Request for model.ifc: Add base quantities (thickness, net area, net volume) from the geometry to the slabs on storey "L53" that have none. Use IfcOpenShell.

First a look at what the model holds.

```python
import ifcopenshell
import ifcopenshell.util.element
import ifcopenshell.util.unit

model = ifcopenshell.open("model.ifc")
print(model.schema)
for unit_type in ("LENGTHUNIT", "AREAUNIT", "VOLUMEUNIT"):
    print(unit_type, ifcopenshell.util.unit.calculate_unit_scale(model, unit_type))
storey = next(s for s in model.by_type("IfcBuildingStorey") if s.Name == "L53")
slabs = [e for e in ifcopenshell.util.element.get_decomposition(storey) if e.is_a("IfcSlab")]
for e in sorted(slabs, key=lambda e: e.id()):
    print(e.id(), e.is_a(), e.Name, list(ifcopenshell.util.element.get_psets(e, qtos_only=True)), sep=" | ")
```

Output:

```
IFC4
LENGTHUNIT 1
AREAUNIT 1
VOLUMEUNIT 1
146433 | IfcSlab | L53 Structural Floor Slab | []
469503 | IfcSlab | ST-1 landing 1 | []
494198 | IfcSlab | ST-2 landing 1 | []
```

```python
import ifcopenshell
import ifcopenshell.api.pset
import ifcopenshell.geom
import ifcopenshell.util.element
import ifcopenshell.util.shape
import ifcopenshell.util.unit

model = ifcopenshell.open("model.ifc")
unit_scale = ifcopenshell.util.unit.calculate_unit_scale(model)
area_scale = ifcopenshell.util.unit.calculate_unit_scale(model, "AREAUNIT")
volume_scale = ifcopenshell.util.unit.calculate_unit_scale(model, "VOLUMEUNIT")
settings = ifcopenshell.geom.settings()

storey = next(s for s in model.by_type("IfcBuildingStorey") if s.Name == "L53")
slabs = [e for e in ifcopenshell.util.element.get_decomposition(storey) if e.is_a("IfcSlab")]

for e in sorted(slabs, key=lambda e: e.id()):
    if ifcopenshell.util.element.get_psets(e, qtos_only=True, should_inherit=False):
        continue
    # Geometry comes back in metres, in the element's own axes.
    shape = ifcopenshell.geom.create_shape(settings, e)
    values = {
        "Width": ifcopenshell.util.shape.get_z(shape.geometry) / unit_scale,
        "NetArea": ifcopenshell.util.shape.get_footprint_area(shape.geometry) / area_scale,
        "NetVolume": ifcopenshell.util.shape.get_volume(shape.geometry) / volume_scale,
    }
    qto = ifcopenshell.api.pset.add_qto(model, product=e, name="Qto_SlabBaseQuantities")
    ifcopenshell.api.pset.edit_qto(model, qto=qto, properties=values)
    print(e.id(), {k: round(v, 3) for k, v in values.items()})

model.write("model_v2.ifc")
```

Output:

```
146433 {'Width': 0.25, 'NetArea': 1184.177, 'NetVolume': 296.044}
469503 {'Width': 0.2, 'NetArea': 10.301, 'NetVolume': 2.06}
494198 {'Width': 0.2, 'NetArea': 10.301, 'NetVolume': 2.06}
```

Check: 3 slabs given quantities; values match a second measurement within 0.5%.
